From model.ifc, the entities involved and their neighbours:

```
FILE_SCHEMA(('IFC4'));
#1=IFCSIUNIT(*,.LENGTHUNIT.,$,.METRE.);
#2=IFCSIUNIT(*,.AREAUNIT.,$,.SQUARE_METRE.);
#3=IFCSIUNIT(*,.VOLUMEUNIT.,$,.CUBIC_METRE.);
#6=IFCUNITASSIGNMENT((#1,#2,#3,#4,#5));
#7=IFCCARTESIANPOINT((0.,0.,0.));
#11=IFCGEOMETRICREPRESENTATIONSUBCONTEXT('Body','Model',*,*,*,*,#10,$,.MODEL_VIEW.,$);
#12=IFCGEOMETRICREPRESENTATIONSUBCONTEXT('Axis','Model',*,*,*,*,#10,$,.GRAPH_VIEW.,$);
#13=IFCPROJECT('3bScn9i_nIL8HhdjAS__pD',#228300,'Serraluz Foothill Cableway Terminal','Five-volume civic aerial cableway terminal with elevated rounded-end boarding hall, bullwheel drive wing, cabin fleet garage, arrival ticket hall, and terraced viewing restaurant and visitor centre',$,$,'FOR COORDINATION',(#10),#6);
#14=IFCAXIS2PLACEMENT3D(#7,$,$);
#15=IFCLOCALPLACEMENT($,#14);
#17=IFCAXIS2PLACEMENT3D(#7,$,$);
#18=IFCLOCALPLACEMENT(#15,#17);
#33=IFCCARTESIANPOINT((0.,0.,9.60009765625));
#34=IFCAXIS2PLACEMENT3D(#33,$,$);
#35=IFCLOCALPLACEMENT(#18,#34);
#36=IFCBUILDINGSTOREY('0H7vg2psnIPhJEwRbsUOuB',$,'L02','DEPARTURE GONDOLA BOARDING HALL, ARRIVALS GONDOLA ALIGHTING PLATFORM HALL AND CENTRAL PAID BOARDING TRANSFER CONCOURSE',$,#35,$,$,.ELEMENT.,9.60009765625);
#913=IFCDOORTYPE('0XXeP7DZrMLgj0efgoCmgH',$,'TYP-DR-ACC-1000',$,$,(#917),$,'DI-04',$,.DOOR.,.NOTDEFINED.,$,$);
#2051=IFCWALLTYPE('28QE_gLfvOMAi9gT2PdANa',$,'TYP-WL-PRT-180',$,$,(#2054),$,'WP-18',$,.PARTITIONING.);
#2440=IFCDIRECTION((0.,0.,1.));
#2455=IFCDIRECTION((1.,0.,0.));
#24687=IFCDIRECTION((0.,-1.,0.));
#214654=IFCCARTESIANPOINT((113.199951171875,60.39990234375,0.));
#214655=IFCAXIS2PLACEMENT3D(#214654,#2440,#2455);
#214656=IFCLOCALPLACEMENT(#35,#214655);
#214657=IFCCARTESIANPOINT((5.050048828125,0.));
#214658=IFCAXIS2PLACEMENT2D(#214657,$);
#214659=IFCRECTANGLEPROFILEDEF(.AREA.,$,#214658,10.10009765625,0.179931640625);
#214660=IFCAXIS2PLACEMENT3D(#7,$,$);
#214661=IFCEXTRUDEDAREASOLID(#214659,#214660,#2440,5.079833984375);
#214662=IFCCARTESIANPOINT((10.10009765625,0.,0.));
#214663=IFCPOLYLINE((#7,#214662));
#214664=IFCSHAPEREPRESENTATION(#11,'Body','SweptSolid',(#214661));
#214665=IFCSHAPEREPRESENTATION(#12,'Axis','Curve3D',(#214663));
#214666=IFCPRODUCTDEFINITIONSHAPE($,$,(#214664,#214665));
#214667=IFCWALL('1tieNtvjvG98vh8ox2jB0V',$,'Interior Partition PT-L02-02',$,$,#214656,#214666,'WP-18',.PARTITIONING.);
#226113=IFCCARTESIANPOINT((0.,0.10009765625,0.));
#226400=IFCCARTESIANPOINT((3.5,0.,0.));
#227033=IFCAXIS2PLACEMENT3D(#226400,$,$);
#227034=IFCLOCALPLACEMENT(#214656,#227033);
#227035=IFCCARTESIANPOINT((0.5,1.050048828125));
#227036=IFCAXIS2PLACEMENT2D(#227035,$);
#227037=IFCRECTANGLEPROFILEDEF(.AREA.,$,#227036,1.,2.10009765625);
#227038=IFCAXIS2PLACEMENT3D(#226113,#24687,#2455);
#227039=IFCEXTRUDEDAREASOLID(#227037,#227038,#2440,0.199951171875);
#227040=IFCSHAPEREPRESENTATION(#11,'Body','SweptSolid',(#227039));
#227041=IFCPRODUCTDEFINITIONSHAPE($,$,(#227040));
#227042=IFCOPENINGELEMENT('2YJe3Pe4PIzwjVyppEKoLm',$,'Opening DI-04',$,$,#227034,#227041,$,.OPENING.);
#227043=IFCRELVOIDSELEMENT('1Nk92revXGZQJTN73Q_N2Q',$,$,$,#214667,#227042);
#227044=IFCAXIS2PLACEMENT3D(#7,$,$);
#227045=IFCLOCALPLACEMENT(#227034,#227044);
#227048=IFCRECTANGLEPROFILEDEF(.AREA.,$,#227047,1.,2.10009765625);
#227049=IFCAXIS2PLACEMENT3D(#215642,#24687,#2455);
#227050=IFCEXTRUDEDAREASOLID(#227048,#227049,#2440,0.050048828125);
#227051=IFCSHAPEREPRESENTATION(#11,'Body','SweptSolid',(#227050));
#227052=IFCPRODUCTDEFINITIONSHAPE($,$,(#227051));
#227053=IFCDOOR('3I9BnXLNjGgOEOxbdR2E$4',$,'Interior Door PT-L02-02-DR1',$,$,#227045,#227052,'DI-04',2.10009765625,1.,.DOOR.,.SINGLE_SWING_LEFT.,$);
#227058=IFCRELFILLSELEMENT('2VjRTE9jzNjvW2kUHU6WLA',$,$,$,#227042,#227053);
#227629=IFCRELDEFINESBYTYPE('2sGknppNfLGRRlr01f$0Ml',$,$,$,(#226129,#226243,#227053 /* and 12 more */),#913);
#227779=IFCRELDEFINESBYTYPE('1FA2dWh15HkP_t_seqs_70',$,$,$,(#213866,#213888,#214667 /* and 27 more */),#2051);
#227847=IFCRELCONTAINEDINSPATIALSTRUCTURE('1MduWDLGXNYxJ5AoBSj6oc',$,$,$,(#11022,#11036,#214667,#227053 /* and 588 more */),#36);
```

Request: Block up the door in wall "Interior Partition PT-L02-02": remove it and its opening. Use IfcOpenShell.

```python
import ifcopenshell
import ifcopenshell.api.feature
import ifcopenshell.api.root
import ifcopenshell.geom
import ifcopenshell.util.shape

model = ifcopenshell.open("model.ifc")
settings = ifcopenshell.geom.settings()


def volume(element):
    """Net volume in cubic metres, openings subtracted."""
    shape = ifcopenshell.geom.create_shape(settings, element)
    return ifcopenshell.util.shape.get_volume(shape.geometry)


door = model.by_guid("3I9BnXLNjGgOEOxbdR2E$4")
opening = door.FillsVoids[0].RelatingOpeningElement
wall = opening.VoidsElements[0].RelatingBuildingElement
before = volume(wall)

ifcopenshell.api.root.remove_product(model, product=door)
ifcopenshell.api.feature.remove_feature(model, feature=opening)

after = volume(wall)

print(f"wall volume {before:.3f} -> {after:.3f} m3")

model.write("model-out.ifc")
```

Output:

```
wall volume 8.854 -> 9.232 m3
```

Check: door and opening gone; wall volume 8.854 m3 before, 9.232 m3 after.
